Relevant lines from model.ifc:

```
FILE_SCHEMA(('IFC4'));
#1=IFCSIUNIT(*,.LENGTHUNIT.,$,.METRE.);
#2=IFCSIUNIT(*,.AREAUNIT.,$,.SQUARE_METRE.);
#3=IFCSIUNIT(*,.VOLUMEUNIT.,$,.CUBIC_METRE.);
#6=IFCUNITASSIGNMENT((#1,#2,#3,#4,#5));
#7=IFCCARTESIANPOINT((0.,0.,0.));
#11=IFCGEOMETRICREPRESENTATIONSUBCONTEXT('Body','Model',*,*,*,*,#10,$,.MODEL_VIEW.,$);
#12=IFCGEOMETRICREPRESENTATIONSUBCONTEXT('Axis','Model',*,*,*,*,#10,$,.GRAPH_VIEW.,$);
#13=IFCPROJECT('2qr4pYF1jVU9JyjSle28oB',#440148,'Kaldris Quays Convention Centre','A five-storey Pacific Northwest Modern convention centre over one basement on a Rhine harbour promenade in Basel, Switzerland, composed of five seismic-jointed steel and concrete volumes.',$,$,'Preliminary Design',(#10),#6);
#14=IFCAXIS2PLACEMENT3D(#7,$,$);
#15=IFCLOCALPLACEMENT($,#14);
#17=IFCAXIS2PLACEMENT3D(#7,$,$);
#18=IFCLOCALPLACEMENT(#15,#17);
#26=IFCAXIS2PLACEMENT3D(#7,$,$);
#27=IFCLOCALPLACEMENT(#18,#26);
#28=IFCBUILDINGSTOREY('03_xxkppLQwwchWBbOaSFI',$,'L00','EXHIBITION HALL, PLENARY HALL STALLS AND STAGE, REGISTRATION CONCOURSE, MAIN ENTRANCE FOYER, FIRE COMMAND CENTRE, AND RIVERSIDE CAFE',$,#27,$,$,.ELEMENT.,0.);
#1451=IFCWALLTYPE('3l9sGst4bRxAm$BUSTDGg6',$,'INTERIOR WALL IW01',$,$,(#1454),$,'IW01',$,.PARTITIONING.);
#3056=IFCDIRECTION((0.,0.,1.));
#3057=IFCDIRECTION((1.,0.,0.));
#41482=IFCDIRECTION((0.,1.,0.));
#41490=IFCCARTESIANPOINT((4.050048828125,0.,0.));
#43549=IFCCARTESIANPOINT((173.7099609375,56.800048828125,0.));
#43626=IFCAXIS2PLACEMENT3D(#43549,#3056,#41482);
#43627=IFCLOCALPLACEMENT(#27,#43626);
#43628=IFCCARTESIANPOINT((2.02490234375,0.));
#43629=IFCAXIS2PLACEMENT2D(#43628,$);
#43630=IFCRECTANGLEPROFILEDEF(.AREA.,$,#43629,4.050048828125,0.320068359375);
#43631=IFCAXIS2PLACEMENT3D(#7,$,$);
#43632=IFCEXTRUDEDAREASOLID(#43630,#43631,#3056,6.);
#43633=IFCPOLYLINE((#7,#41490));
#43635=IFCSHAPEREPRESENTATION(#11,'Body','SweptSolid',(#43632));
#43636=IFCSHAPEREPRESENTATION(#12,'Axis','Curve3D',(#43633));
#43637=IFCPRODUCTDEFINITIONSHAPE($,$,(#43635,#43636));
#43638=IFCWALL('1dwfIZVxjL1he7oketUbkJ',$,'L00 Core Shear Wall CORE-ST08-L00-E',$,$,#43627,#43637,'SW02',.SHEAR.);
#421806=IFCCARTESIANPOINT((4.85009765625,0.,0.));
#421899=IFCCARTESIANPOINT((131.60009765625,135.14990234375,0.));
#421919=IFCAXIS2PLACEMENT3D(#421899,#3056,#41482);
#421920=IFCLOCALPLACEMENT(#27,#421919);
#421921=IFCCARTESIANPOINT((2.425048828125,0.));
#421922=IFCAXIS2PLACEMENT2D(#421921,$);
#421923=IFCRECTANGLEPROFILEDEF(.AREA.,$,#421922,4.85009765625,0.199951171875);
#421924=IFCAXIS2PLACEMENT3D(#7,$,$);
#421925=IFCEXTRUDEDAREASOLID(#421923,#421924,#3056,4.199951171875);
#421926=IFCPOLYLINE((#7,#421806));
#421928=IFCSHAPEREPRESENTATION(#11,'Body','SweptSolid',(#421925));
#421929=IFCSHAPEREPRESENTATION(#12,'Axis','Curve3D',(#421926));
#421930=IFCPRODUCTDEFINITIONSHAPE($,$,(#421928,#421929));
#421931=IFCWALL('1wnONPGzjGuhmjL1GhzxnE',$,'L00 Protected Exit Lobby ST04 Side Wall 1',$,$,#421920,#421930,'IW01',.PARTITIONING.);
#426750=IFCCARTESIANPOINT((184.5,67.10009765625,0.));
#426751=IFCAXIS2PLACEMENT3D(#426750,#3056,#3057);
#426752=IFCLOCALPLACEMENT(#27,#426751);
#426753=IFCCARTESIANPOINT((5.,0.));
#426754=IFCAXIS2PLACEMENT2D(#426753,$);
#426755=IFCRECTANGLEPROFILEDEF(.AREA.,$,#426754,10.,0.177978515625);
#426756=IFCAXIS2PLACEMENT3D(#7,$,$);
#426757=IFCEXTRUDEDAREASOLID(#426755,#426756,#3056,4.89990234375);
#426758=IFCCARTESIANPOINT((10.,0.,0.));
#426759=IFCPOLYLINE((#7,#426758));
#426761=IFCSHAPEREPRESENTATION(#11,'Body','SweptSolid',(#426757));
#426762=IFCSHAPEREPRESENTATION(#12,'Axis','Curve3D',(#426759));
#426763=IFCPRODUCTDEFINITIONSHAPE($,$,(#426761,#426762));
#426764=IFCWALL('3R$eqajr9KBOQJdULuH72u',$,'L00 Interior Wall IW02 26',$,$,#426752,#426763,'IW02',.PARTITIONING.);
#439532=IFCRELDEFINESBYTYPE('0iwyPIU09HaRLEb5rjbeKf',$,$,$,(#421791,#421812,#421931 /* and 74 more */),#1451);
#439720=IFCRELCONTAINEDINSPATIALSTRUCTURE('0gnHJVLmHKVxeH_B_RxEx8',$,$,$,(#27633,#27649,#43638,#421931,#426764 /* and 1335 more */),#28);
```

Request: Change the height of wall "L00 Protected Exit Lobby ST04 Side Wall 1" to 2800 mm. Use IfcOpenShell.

```python
import ifcopenshell
import ifcopenshell.geom
import ifcopenshell.util.representation
import ifcopenshell.util.shape

model = ifcopenshell.open("model.ifc")
settings = ifcopenshell.geom.settings()


def volume(element):
    """Net volume in cubic metres, openings subtracted."""
    shape = ifcopenshell.geom.create_shape(settings, element)
    return ifcopenshell.util.shape.get_volume(shape.geometry)


wall = model.by_guid("1wnONPGzjGuhmjL1GhzxnE")
before = volume(wall)

body = ifcopenshell.util.representation.get_representation(wall, "Model", "Body")
solid = body.Items[0]
old_height = solid.Depth
solid.Depth = 2.8
after = volume(wall)

print(f"height {old_height:g} -> {solid.Depth:g}, volume {before:.3f} -> {after:.3f} m3")

model.write("model_rev.ifc")
```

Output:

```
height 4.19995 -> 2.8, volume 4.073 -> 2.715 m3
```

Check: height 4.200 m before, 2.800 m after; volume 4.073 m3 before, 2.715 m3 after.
